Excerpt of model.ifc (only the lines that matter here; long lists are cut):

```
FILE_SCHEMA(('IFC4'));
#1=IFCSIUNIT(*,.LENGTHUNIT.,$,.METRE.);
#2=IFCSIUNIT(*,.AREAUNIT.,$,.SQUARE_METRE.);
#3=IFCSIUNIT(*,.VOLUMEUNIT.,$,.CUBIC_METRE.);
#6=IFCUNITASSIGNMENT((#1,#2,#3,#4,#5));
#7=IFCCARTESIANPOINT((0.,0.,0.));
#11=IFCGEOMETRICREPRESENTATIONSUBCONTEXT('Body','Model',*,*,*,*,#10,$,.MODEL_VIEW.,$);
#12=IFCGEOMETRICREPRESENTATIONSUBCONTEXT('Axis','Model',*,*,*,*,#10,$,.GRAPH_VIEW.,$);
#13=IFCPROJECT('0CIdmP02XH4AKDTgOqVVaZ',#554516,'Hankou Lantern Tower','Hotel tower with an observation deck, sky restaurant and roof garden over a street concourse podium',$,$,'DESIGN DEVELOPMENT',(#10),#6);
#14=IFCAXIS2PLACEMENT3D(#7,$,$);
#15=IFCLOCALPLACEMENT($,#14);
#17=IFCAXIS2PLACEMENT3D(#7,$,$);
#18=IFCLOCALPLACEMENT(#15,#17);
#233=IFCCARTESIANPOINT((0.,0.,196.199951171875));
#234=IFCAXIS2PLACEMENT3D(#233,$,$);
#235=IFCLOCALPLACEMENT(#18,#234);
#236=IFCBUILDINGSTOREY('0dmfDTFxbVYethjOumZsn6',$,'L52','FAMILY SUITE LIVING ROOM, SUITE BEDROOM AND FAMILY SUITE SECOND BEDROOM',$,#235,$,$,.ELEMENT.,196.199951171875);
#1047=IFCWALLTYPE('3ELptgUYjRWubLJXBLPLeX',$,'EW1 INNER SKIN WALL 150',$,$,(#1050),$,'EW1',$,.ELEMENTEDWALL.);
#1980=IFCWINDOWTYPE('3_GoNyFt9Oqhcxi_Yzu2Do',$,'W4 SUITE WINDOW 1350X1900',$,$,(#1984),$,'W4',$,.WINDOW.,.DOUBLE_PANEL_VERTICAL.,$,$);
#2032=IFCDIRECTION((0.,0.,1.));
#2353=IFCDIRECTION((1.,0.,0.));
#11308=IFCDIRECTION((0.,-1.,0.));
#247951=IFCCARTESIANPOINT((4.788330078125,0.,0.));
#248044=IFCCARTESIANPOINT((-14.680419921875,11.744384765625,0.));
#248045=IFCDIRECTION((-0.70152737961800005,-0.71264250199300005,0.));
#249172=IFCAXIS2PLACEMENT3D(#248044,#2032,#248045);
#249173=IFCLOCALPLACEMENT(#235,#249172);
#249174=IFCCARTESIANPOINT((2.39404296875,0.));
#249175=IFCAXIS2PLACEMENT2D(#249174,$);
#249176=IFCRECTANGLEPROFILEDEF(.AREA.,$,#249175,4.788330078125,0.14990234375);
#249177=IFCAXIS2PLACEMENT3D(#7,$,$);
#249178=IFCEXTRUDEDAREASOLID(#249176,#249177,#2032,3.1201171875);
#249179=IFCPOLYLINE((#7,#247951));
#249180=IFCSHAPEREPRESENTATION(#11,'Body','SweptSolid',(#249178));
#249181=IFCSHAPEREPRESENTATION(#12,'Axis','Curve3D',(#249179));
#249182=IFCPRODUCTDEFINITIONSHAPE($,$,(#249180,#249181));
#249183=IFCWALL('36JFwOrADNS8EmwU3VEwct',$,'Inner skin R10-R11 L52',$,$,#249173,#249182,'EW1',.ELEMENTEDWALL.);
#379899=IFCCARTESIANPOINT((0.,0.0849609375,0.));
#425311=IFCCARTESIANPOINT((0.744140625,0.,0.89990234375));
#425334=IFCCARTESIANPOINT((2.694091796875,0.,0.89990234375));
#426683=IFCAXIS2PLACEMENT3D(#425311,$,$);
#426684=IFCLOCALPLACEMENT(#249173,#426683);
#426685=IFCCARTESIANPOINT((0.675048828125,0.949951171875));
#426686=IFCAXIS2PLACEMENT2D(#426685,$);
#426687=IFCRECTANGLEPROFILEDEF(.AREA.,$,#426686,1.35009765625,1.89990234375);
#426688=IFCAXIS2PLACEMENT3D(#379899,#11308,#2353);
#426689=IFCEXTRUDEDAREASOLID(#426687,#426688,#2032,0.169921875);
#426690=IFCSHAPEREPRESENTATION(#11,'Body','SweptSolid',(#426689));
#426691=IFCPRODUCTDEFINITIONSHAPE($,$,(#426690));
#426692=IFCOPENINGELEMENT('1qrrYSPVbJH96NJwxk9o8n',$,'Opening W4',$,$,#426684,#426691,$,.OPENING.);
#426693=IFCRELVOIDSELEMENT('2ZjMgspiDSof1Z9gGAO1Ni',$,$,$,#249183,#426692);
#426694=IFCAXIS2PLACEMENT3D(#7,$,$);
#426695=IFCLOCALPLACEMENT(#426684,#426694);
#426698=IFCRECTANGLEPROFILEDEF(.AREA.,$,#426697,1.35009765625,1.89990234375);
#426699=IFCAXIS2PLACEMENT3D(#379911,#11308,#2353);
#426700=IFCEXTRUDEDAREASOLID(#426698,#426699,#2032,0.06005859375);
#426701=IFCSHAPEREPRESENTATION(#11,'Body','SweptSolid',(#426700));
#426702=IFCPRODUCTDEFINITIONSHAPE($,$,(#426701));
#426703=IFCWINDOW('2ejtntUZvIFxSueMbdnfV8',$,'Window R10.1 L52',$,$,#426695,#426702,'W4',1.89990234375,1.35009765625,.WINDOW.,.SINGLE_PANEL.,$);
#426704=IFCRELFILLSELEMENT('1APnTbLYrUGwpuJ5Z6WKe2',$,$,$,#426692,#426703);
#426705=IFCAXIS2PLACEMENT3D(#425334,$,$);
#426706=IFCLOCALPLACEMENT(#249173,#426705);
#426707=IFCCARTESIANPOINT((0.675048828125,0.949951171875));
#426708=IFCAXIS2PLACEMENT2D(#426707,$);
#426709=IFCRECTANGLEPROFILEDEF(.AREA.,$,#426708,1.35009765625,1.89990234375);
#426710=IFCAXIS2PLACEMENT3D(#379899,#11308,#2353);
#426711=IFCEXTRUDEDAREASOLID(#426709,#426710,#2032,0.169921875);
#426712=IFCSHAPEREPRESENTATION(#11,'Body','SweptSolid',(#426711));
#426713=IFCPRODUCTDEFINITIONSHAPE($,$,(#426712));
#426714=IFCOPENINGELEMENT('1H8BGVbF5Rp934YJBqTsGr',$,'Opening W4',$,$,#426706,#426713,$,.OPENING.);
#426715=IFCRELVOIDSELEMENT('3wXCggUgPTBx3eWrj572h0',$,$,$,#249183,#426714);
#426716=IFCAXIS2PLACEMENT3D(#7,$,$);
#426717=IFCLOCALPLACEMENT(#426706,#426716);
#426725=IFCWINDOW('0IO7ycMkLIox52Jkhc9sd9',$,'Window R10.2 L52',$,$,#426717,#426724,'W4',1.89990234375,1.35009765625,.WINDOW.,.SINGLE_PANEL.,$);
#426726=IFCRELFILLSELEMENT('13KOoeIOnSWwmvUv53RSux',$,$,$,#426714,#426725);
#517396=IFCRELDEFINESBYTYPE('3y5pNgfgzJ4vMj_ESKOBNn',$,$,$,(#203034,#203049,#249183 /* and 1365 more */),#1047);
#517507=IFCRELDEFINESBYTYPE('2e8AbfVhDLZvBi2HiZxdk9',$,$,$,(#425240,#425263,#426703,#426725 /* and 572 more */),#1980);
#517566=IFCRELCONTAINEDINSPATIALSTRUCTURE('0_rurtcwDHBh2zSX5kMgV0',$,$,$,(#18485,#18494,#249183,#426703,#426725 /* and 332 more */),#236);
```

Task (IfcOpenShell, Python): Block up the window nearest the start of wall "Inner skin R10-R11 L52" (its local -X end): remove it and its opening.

```python
import ifcopenshell
import ifcopenshell.api.feature
import ifcopenshell.api.root
import ifcopenshell.geom
import ifcopenshell.util.shape

model = ifcopenshell.open("model.ifc")
settings = ifcopenshell.geom.settings()


def volume(element):
    """Net volume in cubic metres, openings subtracted."""
    shape = ifcopenshell.geom.create_shape(settings, element)
    return ifcopenshell.util.shape.get_volume(shape.geometry)


window = model.by_id(426703)
opening = window.FillsVoids[0].RelatingOpeningElement
wall = opening.VoidsElements[0].RelatingBuildingElement
before = volume(wall)

ifcopenshell.api.root.remove_product(model, product=window)
ifcopenshell.api.feature.remove_feature(model, feature=opening)

after = volume(wall)

print(f"wall volume {before:.3f} -> {after:.3f} m3")

model.write("model_edited.ifc")
```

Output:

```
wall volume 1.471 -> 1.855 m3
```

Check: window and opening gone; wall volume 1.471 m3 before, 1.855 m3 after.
